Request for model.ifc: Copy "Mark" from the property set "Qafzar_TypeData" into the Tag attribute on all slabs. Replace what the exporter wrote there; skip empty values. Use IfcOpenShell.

First a look at what the model holds.

```python
import ifcopenshell
import ifcopenshell.util.element

model = ifcopenshell.open("model.ifc")
print(model.schema)
slabs = model.by_type("IfcSlab")
print(len(slabs), "slabs")
for e in slabs[:8]:
    source = ifcopenshell.util.element.get_pset(e, "Qafzar_TypeData", "Mark")
    target = e.Tag
    print(e.id(), repr(source), repr(target), sep=" | ")
```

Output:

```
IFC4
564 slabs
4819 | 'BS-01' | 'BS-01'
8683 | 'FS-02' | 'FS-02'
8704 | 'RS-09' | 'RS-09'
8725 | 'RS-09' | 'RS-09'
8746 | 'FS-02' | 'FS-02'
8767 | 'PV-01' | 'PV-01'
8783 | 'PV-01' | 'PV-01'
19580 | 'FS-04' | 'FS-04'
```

```python
import ifcopenshell
import ifcopenshell.util.element

model = ifcopenshell.open("model.ifc")

count = 0
for e in model.by_type("IfcSlab"):
    value = ifcopenshell.util.element.get_pset(e, "Qafzar_TypeData", "Mark")
    current = e.Tag
    if not value or not value.strip() or current == value:
        continue
    e.Tag = value
    count += 1

print(count, "slabs updated")

model.write("model-out.ifc")
```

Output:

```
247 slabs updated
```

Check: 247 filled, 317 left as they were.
